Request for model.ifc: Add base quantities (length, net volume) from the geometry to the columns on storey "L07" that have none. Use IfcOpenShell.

First a look at what the model holds.

```python
import ifcopenshell
import ifcopenshell.util.element
import ifcopenshell.util.unit

model = ifcopenshell.open("model.ifc")
print(model.schema)
for unit_type in ("LENGTHUNIT", "AREAUNIT", "VOLUMEUNIT"):
    print(unit_type, ifcopenshell.util.unit.calculate_unit_scale(model, unit_type))
storey = next(s for s in model.by_type("IfcBuildingStorey") if s.Name == "L07")
columns = [e for e in ifcopenshell.util.element.get_decomposition(storey) if e.is_a("IfcColumn")]
for e in sorted(columns, key=lambda e: e.id()):
    print(e.id(), e.is_a(), e.Name, list(ifcopenshell.util.element.get_psets(e, qtos_only=True)), sep=" | ")
```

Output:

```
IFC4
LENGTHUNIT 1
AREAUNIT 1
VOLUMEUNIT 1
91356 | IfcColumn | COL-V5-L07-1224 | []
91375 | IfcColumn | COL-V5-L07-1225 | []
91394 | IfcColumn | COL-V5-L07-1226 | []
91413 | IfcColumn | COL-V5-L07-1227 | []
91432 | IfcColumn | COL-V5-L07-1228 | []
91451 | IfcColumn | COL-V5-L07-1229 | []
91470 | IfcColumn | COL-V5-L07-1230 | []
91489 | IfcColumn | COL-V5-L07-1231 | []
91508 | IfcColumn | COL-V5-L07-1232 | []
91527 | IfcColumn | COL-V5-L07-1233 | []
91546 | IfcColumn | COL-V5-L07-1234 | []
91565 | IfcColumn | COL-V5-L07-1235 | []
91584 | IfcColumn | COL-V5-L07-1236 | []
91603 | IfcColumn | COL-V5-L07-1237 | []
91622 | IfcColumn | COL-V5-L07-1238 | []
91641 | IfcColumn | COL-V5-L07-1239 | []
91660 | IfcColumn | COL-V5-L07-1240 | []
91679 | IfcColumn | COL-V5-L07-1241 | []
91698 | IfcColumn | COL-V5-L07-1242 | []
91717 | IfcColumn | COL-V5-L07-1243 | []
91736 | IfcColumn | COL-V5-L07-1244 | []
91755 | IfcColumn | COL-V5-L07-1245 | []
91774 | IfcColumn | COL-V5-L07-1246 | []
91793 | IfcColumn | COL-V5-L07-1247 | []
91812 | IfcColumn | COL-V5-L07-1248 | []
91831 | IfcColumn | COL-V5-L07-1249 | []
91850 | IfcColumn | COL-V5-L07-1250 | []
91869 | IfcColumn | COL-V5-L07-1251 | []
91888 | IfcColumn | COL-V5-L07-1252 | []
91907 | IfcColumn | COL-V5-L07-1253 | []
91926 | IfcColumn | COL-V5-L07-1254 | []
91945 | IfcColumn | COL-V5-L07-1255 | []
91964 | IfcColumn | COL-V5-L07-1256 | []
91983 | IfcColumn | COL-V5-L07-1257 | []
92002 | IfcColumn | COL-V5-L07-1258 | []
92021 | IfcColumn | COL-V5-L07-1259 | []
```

```python
import ifcopenshell
import ifcopenshell.api.pset
import ifcopenshell.geom
import ifcopenshell.util.element
import ifcopenshell.util.shape
import ifcopenshell.util.unit

model = ifcopenshell.open("model.ifc")
unit_scale = ifcopenshell.util.unit.calculate_unit_scale(model)
volume_scale = ifcopenshell.util.unit.calculate_unit_scale(model, "VOLUMEUNIT")
settings = ifcopenshell.geom.settings()

storey = next(s for s in model.by_type("IfcBuildingStorey") if s.Name == "L07")
columns = [e for e in ifcopenshell.util.element.get_decomposition(storey) if e.is_a("IfcColumn")]

for e in sorted(columns, key=lambda e: e.id()):
    if ifcopenshell.util.element.get_psets(e, qtos_only=True, should_inherit=False):
        continue
    # Geometry comes back in metres, in the element's own axes.
    shape = ifcopenshell.geom.create_shape(settings, e)
    values = {
        "Length": ifcopenshell.util.shape.get_z(shape.geometry) / unit_scale,
        "NetVolume": ifcopenshell.util.shape.get_volume(shape.geometry) / volume_scale,
    }
    qto = ifcopenshell.api.pset.add_qto(model, product=e, name="Qto_ColumnBaseQuantities")
    ifcopenshell.api.pset.edit_qto(model, qto=qto, properties=values)
    print(e.id(), {k: round(v, 3) for k, v in values.items()})

model.write("model_updated.ifc")
```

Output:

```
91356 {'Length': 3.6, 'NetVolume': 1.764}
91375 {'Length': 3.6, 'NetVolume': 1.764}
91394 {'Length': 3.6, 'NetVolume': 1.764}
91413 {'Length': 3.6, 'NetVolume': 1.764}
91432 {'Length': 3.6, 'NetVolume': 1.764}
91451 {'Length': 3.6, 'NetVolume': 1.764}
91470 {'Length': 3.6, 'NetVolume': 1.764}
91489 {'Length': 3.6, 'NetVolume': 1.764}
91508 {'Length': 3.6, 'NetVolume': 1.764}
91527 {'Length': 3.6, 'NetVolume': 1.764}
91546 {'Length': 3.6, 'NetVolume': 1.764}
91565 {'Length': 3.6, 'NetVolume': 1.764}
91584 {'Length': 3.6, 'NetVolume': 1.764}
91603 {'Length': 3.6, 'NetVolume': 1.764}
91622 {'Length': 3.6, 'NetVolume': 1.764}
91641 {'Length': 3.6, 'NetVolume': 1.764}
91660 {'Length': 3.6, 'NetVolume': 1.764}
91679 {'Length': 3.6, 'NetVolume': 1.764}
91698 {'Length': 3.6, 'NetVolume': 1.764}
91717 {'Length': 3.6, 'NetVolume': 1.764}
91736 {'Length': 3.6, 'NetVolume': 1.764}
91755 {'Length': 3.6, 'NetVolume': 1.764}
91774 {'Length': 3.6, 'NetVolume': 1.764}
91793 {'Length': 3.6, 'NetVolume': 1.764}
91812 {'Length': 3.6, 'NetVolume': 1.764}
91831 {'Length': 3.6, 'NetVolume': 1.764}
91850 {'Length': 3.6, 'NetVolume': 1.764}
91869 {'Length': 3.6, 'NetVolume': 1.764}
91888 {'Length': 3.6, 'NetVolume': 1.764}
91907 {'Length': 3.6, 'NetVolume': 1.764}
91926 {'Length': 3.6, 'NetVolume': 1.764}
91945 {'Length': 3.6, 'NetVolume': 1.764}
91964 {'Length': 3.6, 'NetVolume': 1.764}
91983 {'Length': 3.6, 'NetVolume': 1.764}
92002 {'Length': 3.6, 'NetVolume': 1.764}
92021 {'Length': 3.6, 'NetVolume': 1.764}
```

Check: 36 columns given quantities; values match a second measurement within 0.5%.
